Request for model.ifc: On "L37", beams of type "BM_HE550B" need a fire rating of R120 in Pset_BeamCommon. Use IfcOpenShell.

First a look at what the model holds.

```python
import ifcopenshell
import ifcopenshell.util.element

model = ifcopenshell.open("model.ifc")
print(model.schema)
storey = next(s for s in model.by_type("IfcBuildingStorey") if s.Name == "L37")
beams = [e for e in ifcopenshell.util.element.get_decomposition(storey) if e.is_a("IfcBeam")]
seen = {}
for e in beams:
    element_type = ifcopenshell.util.element.get_type(e)
    key = (element_type.Name if element_type != e and element_type else None, ifcopenshell.util.element.get_pset(e, "Pset_BeamCommon", "FireRating"))
    seen[key] = seen.get(key, 0) + 1
for (name, value), count in sorted(seen.items(), key=str):
    print(count, "x", name, "|", value)
```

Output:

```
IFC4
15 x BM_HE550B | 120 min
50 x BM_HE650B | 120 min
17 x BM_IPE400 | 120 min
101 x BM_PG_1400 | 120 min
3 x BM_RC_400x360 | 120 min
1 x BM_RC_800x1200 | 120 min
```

```python
import ifcopenshell
import ifcopenshell.api.pset
import ifcopenshell.util.element

model = ifcopenshell.open("model.ifc")

storey = next(s for s in model.by_type("IfcBuildingStorey") if s.Name == "L37")
beams = [e for e in ifcopenshell.util.element.get_decomposition(storey) if e.is_a("IfcBeam")]

count = 0
for e in beams:
    element_type = ifcopenshell.util.element.get_type(e)
    if element_type in (None, e) or element_type.Name != "BM_HE550B":
        continue
    found = ifcopenshell.util.element.get_pset(e, "Pset_BeamCommon", should_inherit=False)
    if found:
        pset = model.by_id(found["id"])
        if len(ifcopenshell.util.element.get_elements_by_pset(pset)) > 1:
            pset = ifcopenshell.api.pset.unshare_pset(model, products=[e], pset=pset)[0]
    else:
        pset = ifcopenshell.api.pset.add_pset(model, product=e, name="Pset_BeamCommon")
    ifcopenshell.api.pset.edit_pset(model, pset=pset, properties={"FireRating": "R120"})
    count += 1

print(count, "beams updated")

model.write("model_edited.ifc")
```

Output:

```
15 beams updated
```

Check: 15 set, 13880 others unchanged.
